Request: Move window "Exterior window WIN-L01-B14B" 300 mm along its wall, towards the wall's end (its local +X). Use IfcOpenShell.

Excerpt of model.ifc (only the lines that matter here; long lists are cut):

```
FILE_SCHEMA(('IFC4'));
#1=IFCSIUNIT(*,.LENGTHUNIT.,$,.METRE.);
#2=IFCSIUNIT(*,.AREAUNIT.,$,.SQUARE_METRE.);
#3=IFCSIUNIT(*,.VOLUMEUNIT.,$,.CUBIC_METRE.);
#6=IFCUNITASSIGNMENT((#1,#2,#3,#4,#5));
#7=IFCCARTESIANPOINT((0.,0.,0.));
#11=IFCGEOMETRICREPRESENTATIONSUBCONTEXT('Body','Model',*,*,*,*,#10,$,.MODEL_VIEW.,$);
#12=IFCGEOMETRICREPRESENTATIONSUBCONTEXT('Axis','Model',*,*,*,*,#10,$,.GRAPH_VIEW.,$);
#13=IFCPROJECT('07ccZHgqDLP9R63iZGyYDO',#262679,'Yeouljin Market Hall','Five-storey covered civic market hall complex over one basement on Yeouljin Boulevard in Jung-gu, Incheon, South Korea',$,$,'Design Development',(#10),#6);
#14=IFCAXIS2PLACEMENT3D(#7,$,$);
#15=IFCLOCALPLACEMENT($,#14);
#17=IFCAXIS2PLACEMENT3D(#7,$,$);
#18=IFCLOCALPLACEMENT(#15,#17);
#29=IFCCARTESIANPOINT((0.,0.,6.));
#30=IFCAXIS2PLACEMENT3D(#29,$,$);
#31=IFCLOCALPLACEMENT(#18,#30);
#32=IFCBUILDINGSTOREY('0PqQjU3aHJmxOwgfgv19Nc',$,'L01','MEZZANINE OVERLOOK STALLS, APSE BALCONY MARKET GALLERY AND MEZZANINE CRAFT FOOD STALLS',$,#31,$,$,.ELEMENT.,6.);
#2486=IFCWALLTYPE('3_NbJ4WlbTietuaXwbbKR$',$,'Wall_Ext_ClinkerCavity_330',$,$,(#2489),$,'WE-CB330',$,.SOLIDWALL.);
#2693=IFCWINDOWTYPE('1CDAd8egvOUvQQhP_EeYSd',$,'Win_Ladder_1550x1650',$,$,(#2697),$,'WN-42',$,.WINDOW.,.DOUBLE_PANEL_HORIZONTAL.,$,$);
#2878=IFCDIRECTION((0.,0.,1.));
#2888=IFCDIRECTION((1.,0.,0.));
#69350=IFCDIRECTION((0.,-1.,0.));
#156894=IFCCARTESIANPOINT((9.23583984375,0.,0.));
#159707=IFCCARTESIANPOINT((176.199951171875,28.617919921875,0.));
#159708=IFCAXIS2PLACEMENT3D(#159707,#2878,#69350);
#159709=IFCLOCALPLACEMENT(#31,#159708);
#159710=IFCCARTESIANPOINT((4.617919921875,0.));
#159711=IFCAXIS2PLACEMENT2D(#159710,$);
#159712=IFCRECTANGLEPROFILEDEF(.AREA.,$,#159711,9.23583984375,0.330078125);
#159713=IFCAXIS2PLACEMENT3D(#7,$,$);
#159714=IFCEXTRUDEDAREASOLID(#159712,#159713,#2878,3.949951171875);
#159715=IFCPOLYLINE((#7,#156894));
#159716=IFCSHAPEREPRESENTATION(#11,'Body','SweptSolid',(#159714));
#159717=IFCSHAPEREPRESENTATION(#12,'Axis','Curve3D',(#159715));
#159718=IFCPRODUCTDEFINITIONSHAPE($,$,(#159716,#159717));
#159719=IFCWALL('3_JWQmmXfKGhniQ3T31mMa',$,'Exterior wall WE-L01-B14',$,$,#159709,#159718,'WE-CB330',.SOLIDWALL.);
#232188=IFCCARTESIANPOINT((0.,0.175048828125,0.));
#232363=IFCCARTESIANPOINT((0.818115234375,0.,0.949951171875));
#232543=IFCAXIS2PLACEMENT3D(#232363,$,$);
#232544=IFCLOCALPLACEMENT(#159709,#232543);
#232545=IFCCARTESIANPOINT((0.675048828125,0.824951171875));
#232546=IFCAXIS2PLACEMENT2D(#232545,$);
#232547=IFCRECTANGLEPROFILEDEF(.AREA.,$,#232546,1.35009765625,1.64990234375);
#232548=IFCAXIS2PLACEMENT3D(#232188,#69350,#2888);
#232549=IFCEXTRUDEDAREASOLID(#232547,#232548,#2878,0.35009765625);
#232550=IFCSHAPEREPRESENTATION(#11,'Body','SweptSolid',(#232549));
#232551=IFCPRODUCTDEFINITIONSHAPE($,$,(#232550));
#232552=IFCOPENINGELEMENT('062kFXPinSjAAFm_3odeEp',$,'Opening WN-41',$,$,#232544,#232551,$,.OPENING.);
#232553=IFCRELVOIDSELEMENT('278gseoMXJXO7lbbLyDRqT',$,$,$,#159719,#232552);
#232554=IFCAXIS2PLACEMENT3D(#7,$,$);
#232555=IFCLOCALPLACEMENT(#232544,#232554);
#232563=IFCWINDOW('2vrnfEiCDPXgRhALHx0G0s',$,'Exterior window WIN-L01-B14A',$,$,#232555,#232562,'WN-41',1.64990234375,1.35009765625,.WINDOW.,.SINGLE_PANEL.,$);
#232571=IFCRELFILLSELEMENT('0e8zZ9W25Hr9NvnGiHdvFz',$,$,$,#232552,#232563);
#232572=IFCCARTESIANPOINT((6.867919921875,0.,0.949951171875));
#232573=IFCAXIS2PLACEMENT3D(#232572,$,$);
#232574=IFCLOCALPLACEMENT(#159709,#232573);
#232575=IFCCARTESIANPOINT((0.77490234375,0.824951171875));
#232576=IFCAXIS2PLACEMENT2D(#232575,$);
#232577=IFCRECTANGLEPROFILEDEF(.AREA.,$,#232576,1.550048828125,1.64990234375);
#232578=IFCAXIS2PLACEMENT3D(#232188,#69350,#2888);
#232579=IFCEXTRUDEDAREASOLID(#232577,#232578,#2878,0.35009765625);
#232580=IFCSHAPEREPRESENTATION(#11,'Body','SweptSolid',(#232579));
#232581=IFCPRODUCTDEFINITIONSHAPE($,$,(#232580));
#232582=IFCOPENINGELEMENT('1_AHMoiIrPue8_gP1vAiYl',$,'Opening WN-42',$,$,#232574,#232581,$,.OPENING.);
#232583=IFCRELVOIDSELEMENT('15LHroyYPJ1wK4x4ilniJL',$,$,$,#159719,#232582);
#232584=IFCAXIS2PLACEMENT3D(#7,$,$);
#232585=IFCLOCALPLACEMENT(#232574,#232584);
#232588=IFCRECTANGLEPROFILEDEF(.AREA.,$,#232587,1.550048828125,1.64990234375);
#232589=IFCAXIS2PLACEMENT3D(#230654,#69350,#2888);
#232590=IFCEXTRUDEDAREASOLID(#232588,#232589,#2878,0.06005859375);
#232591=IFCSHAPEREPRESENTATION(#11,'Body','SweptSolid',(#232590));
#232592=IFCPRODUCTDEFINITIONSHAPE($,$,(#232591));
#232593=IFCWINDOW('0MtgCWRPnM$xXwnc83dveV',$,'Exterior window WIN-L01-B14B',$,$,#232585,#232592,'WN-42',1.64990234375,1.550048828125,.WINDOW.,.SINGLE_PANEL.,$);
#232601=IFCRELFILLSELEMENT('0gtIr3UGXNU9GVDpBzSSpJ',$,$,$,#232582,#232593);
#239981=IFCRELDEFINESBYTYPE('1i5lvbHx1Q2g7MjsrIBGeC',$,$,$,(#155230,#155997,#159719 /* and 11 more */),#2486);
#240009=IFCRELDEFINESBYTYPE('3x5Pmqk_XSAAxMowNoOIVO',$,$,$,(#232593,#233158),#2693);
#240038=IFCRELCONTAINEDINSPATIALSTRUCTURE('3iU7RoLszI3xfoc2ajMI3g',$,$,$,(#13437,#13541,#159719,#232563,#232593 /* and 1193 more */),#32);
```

```python
import ifcopenshell
import ifcopenshell.api.geometry
import ifcopenshell.util.placement
import ifcopenshell.util.unit

model = ifcopenshell.open("model.ifc")
unit_scale = ifcopenshell.util.unit.calculate_unit_scale(model)

window = model.by_guid("0MtgCWRPnM$xXwnc83dveV")
opening = window.FillsVoids[0].RelatingOpeningElement
wall = opening.VoidsElements[0].RelatingBuildingElement

wall_matrix = ifcopenshell.util.placement.get_local_placement(wall.ObjectPlacement)
shift = wall_matrix[:3, 0] * 0.3 / unit_scale
before = ifcopenshell.util.placement.get_local_placement(window.ObjectPlacement)[:3, 3].copy()

# The window is placed relative to its opening, so it follows when the opening moves.
matrix = ifcopenshell.util.placement.get_local_placement(opening.ObjectPlacement)
matrix[:3, 3] += shift
ifcopenshell.api.geometry.edit_object_placement(
    model, product=opening, matrix=matrix, is_si=False, should_transform_children=True
)

after = ifcopenshell.util.placement.get_local_placement(window.ObjectPlacement)[:3, 3]
print("window moved by", (after - before).round(3) + 0.0)

model.write("model_edited.ifc")
```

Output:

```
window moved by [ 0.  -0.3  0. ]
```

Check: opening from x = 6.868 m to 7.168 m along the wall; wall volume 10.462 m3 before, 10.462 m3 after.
